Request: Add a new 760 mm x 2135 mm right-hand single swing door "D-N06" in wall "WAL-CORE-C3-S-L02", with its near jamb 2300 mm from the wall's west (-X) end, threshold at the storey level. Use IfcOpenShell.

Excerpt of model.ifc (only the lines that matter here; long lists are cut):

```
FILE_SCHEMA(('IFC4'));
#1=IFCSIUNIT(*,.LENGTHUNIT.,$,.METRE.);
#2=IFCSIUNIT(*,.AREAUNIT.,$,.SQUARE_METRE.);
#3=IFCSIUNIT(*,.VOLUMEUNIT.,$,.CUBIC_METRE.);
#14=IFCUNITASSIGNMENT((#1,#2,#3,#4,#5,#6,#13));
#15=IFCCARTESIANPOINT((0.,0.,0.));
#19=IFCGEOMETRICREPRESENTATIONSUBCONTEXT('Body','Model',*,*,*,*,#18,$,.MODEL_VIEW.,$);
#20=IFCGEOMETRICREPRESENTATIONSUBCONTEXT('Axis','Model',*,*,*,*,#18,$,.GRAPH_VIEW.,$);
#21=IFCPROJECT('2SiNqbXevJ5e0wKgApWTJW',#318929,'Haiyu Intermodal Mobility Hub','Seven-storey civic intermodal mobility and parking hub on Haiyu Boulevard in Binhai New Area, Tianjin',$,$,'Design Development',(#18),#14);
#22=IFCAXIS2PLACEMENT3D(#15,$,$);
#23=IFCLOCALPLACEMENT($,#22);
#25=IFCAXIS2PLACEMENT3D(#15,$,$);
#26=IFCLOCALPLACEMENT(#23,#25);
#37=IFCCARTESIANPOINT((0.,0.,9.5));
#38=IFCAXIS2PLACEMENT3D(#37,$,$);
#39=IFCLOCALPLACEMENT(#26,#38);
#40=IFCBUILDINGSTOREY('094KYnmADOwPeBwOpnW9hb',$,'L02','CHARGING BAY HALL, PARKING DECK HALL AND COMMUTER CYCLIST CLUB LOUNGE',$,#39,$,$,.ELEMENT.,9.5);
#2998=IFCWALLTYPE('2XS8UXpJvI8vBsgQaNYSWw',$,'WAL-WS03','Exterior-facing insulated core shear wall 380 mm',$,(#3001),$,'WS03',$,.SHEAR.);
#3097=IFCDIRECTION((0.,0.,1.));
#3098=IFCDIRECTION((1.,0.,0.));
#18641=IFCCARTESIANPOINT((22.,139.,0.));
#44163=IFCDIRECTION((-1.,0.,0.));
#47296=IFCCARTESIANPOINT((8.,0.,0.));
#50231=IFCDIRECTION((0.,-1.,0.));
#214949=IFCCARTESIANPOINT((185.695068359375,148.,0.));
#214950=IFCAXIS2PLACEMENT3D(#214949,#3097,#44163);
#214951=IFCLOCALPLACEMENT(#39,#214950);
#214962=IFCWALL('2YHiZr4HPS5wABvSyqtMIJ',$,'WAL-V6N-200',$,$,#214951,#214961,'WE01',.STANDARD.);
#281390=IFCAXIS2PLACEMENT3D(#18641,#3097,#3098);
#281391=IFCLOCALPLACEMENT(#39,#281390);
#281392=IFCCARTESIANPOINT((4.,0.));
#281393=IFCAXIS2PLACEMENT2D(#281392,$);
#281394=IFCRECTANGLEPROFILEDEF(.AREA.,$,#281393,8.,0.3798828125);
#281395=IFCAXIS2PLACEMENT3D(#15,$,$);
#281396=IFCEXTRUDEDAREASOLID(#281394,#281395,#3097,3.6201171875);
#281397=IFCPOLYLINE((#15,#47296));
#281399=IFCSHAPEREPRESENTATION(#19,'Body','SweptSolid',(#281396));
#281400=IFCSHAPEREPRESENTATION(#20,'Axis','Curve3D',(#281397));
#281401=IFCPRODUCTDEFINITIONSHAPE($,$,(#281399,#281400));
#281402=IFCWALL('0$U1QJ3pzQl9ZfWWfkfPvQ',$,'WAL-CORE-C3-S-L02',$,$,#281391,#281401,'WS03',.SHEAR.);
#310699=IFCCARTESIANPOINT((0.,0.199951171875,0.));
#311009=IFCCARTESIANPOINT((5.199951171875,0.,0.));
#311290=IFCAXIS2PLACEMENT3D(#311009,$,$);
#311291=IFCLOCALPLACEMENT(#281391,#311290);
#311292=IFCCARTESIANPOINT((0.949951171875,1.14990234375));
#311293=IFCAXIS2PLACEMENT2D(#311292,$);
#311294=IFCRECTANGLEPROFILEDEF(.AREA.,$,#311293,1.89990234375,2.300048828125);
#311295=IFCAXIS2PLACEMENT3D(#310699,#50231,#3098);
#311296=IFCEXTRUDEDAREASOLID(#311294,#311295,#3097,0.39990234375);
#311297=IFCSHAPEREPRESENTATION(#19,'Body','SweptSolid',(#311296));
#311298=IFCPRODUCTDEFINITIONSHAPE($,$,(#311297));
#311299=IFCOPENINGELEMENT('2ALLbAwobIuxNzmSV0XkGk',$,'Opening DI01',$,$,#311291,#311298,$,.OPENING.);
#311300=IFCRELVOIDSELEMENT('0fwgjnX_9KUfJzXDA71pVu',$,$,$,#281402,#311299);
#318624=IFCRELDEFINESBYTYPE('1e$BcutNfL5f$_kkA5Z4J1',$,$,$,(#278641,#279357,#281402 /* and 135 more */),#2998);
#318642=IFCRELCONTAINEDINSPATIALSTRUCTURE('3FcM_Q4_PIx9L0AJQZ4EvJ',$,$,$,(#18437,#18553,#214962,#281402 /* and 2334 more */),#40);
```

```python
import numpy as np
import ifcopenshell
import ifcopenshell.api.feature
import ifcopenshell.api.geometry
import ifcopenshell.api.root
import ifcopenshell.api.spatial
import ifcopenshell.geom
import ifcopenshell.util.element
import ifcopenshell.util.placement
import ifcopenshell.util.representation
import ifcopenshell.util.shape
import ifcopenshell.util.unit

model = ifcopenshell.open("model.ifc")
unit_scale = ifcopenshell.util.unit.calculate_unit_scale(model)
settings = ifcopenshell.geom.settings()


def volume(element):
    """Net volume in cubic metres, openings subtracted."""
    shape = ifcopenshell.geom.create_shape(settings, element)
    return ifcopenshell.util.shape.get_volume(shape.geometry)


wall = model.by_id(281402)
storey = ifcopenshell.util.element.get_container(wall, ifc_class="IfcBuildingStorey")
context = ifcopenshell.util.representation.get_context(model, "Model", "Body", "MODEL_VIEW")
before = volume(wall)

width, height, from_end, sill = 0.76, 2.135, 2.3, 0.0  # metres

# The wall runs along its own X axis, and the end named is its -X end.
wall_shape = ifcopenshell.geom.create_shape(settings, wall)
x, y, z = ifcopenshell.util.shape.get_vertices(wall_shape.geometry).T
start = x.min() + from_end
face, thickness = float(y.min()), float(y.max() - y.min())
wall_matrix = ifcopenshell.util.placement.get_local_placement(wall.ObjectPlacement)
level = ifcopenshell.util.placement.get_local_placement(storey.ObjectPlacement)[2, 3]


def in_wall(x, y):
    """Placement at x, y metres in the wall's axes, at sill height."""
    matrix = wall_matrix.copy()
    matrix[:, 3] = wall_matrix @ np.array([x / unit_scale, y / unit_scale, 0.0, 1.0])
    matrix[2, 3] = level + sill / unit_scale
    return matrix


# Opening: a box that overshoots both wall faces by 50 mm.
opening = ifcopenshell.api.root.create_entity(model, ifc_class="IfcOpeningElement", predefined_type="OPENING")
box = ifcopenshell.api.geometry.add_wall_representation(
    model, context=context, length=width, height=height, thickness=thickness + 0.1
)
ifcopenshell.api.geometry.assign_representation(model, product=opening, representation=box)
ifcopenshell.api.geometry.edit_object_placement(model, product=opening, matrix=in_wall(start, face - 0.05), is_si=False)
ifcopenshell.api.feature.add_feature(model, feature=opening, element=wall)

door = ifcopenshell.api.root.create_entity(model, ifc_class="IfcDoor", name="D-N06", predefined_type="DOOR")
door.OverallWidth, door.OverallHeight = width / unit_scale, height / unit_scale
door.OperationType = "SINGLE_SWING_RIGHT"
body = ifcopenshell.api.geometry.add_door_representation(
    model,
    context=context,
    overall_width=door.OverallWidth,
    overall_height=door.OverallHeight,
    operation_type="SINGLE_SWING_RIGHT",
    lining_properties={"LiningDepth": thickness / unit_scale, "ThresholdDepth": thickness / unit_scale},
)
ifcopenshell.api.geometry.assign_representation(model, product=door, representation=body)
ifcopenshell.api.spatial.assign_container(model, products=[door], relating_structure=storey)
ifcopenshell.api.feature.add_filling(model, opening=opening, element=door)

# The lining spans the wall, so the door starts at the wall face.
ifcopenshell.api.geometry.edit_object_placement(model, product=door, matrix=in_wall(start, face), is_si=False)

after = volume(wall)

print(f"wall volume {before:.3f} -> {after:.3f} m3")

model.write("model_updated.ifc")
```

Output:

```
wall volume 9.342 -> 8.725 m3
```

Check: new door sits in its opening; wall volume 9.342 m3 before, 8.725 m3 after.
